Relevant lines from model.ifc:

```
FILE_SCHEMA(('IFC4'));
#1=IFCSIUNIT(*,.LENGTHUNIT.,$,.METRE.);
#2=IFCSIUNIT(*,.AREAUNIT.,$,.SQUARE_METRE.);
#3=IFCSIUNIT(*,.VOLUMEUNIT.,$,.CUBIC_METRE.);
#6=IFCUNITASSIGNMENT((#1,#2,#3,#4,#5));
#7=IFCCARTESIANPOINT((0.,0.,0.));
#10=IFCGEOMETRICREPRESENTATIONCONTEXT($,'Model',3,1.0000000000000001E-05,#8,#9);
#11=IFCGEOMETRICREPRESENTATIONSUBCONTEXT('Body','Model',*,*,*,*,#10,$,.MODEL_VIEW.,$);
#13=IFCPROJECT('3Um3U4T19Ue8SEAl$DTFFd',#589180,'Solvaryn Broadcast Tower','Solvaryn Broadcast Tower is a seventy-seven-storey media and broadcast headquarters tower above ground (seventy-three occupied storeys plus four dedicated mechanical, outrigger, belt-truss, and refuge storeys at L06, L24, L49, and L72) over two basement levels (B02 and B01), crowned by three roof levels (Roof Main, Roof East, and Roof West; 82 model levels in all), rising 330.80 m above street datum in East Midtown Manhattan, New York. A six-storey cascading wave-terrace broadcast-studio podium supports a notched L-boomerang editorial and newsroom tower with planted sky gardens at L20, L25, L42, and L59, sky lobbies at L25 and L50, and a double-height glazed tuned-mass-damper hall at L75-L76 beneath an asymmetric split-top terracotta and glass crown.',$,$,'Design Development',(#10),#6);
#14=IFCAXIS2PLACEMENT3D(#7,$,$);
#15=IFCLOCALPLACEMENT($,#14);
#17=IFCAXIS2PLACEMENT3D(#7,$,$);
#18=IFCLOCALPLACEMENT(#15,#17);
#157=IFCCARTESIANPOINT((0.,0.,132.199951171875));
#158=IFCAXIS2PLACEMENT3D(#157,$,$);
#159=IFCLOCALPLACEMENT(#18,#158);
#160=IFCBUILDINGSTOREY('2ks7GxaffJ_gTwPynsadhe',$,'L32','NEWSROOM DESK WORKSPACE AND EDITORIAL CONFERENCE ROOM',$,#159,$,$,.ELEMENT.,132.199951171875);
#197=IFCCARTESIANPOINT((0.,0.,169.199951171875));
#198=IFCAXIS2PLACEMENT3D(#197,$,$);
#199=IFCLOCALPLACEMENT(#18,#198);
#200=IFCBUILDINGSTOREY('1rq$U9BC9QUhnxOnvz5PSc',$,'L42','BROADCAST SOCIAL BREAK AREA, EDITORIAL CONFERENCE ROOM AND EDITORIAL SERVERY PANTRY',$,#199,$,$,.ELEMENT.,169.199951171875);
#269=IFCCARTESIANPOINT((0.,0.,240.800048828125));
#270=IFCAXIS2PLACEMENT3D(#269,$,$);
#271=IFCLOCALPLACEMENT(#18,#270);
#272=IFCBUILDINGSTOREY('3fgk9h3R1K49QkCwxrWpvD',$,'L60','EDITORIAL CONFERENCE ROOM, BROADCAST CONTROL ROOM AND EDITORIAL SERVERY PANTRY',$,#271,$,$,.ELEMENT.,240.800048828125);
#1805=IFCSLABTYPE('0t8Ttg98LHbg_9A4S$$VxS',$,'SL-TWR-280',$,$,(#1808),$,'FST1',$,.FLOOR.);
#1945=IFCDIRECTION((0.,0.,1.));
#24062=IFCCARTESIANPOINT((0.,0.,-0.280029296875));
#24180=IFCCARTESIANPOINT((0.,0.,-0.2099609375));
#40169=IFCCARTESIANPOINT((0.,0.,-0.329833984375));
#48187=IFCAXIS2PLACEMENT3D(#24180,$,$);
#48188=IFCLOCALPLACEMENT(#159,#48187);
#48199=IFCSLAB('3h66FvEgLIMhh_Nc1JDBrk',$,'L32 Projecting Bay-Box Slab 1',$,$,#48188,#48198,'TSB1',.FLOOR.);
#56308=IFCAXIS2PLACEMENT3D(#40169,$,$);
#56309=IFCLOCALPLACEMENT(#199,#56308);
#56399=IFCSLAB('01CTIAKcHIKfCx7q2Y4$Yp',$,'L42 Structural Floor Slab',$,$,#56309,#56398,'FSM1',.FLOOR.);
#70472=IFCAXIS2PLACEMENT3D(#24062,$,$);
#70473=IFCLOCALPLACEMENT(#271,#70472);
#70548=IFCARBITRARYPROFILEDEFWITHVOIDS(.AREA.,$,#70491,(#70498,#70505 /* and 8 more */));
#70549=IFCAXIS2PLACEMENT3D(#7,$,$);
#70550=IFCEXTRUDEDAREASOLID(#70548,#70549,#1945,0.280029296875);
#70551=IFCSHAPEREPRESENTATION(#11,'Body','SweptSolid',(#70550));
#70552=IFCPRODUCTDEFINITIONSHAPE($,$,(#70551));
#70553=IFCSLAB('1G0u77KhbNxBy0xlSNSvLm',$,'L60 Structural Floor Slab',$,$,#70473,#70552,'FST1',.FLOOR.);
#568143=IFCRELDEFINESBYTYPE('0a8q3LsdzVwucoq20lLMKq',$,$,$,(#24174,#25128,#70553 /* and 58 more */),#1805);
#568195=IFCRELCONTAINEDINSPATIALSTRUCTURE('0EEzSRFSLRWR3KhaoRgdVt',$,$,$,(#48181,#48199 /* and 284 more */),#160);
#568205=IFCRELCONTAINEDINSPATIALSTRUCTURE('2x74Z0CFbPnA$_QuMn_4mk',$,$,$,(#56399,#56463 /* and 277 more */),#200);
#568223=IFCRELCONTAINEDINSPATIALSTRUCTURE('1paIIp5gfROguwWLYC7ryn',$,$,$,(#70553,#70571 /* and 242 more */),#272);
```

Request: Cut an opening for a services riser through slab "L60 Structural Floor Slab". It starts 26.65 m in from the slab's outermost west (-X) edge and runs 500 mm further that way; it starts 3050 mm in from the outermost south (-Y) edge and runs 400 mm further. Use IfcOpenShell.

```python
import numpy as np
import ifcopenshell
import ifcopenshell.api.feature
import ifcopenshell.api.geometry
import ifcopenshell.api.root
import ifcopenshell.geom
import ifcopenshell.util.placement
import ifcopenshell.util.representation
import ifcopenshell.util.shape
import ifcopenshell.util.unit

model = ifcopenshell.open("model.ifc")
unit_scale = ifcopenshell.util.unit.calculate_unit_scale(model)
settings = ifcopenshell.geom.settings()


def volume(element):
    """Net volume in cubic metres, openings subtracted."""
    shape = ifcopenshell.geom.create_shape(settings, element)
    return ifcopenshell.util.shape.get_volume(shape.geometry)


slab = model.by_guid("1G0u77KhbNxBy0xlSNSvLm")
before = volume(slab)

# Extent in the slab's own axes, in metres. The edges named are its -X and -Y sides.
slab_shape = ifcopenshell.geom.create_shape(settings, slab)
vertices = ifcopenshell.util.shape.get_vertices(slab_shape.geometry)
x_min, y_min, bottom = vertices.min(axis=0)
top = vertices[:, 2].max()

opening = ifcopenshell.api.root.create_entity(model, ifc_class="IfcOpeningElement", name="Services riser opening", predefined_type="OPENING")
context = ifcopenshell.util.representation.get_context(model, "Model", "Body", "MODEL_VIEW")
width, depth = 0.5, 0.4
outline = [(0.0, 0.0), (width, 0.0), (width, depth), (0.0, depth), (0.0, 0.0)]
# Overshoot both faces by 50 mm so the cut is clean.
shape = ifcopenshell.api.geometry.add_slab_representation(
    model, context=context, depth=top - bottom + 0.1, polyline=outline
)
ifcopenshell.api.geometry.assign_representation(model, product=opening, representation=shape)

matrix = ifcopenshell.util.placement.get_local_placement(slab.ObjectPlacement)
matrix[:, 3] = matrix @ np.append(np.array([x_min + 26.65, y_min + 3.05, bottom - 0.05]) / unit_scale, 1.0)
ifcopenshell.api.geometry.edit_object_placement(model, product=opening, matrix=matrix, is_si=False)
ifcopenshell.api.feature.add_feature(model, feature=opening, element=slab)

after = volume(slab)

print(f"slab volume {before:.3f} -> {after:.3f} m3")

model.write("model_edited.ifc")
```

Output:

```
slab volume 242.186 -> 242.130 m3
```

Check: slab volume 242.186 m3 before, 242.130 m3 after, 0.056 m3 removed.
